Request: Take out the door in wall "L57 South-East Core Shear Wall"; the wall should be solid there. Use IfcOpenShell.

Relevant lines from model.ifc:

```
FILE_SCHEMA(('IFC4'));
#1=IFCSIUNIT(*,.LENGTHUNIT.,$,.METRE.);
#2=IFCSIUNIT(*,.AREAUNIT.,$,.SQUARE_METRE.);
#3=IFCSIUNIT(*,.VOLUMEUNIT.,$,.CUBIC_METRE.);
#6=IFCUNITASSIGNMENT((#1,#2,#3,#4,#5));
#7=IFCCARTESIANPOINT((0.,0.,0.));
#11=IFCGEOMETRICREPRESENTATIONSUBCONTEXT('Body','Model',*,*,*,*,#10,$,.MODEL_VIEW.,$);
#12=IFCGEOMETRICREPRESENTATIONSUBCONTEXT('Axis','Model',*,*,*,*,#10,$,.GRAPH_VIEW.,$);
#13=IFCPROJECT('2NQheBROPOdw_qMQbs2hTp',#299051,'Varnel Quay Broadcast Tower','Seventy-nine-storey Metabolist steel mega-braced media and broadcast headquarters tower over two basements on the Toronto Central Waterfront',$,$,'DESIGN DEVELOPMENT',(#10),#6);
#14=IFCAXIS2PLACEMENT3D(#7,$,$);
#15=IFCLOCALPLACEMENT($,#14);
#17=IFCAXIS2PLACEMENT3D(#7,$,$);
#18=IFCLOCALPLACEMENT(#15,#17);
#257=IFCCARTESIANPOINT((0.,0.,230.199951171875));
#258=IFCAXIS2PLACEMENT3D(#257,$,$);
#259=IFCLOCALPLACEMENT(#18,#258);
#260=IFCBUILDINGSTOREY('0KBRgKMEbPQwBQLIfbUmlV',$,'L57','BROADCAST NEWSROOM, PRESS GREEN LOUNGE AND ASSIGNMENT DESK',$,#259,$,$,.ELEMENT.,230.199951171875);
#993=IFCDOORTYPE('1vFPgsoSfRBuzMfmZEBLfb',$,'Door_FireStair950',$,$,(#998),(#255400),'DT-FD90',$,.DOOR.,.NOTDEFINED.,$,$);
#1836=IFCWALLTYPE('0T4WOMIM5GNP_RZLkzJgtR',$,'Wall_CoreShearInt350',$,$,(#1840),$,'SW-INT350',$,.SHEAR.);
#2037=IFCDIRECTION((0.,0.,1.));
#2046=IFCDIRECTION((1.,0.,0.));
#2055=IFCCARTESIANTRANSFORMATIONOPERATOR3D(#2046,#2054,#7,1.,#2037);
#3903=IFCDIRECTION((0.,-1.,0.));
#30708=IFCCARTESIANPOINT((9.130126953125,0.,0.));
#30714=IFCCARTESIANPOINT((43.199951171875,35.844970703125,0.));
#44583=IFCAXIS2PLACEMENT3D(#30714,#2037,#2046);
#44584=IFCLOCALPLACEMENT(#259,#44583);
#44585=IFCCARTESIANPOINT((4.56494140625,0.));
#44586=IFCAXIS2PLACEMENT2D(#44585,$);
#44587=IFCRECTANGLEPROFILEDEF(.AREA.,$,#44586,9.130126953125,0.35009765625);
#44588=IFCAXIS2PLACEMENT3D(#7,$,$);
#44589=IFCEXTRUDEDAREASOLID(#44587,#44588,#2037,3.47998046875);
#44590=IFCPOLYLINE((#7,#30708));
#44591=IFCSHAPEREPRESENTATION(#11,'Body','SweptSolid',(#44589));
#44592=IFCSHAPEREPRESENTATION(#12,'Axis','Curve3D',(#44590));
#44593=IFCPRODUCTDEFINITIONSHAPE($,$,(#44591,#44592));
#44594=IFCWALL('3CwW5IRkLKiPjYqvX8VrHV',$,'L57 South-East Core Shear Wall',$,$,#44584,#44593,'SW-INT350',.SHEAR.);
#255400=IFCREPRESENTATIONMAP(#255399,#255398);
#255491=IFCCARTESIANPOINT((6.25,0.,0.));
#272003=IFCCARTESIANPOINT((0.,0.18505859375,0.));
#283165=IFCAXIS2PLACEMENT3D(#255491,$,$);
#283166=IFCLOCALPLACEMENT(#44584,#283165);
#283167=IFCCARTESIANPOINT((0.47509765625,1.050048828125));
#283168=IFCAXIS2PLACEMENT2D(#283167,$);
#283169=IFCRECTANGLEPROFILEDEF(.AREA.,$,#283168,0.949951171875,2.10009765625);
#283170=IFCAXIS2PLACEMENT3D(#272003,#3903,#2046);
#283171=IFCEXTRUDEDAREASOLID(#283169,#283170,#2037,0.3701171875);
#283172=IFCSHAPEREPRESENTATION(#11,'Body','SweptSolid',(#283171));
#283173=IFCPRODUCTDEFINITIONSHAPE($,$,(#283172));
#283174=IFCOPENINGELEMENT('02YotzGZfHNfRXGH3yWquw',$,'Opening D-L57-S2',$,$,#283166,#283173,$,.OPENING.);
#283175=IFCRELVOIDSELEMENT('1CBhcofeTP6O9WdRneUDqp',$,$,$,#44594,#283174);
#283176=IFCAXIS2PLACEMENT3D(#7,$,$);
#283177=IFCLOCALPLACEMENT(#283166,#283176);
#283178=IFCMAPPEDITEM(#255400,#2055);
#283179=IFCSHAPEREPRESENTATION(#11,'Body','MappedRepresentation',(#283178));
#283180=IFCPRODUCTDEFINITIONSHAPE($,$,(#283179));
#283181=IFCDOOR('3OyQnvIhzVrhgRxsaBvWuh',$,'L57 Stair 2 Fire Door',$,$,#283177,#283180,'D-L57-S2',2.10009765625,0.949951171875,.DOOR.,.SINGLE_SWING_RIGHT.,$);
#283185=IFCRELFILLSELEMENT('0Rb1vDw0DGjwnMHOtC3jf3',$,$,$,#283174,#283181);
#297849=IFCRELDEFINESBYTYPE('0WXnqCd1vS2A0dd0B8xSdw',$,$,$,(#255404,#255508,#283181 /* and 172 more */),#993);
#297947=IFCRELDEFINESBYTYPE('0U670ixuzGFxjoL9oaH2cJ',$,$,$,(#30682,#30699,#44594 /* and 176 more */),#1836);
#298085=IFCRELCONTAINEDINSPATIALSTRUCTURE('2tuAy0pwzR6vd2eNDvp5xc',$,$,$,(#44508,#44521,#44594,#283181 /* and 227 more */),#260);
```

```python
import ifcopenshell
import ifcopenshell.api.feature
import ifcopenshell.api.root
import ifcopenshell.geom
import ifcopenshell.util.shape

model = ifcopenshell.open("model.ifc")
settings = ifcopenshell.geom.settings()


def volume(element):
    """Net volume in cubic metres, openings subtracted."""
    shape = ifcopenshell.geom.create_shape(settings, element)
    return ifcopenshell.util.shape.get_volume(shape.geometry)


door = model.by_guid("3OyQnvIhzVrhgRxsaBvWuh")
opening = door.FillsVoids[0].RelatingOpeningElement
wall = opening.VoidsElements[0].RelatingBuildingElement
before = volume(wall)

ifcopenshell.api.root.remove_product(model, product=door)
ifcopenshell.api.feature.remove_feature(model, feature=opening)

after = volume(wall)

print(f"wall volume {before:.3f} -> {after:.3f} m3")

model.write("model_rev.ifc")
```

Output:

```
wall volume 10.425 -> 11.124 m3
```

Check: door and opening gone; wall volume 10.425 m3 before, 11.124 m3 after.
